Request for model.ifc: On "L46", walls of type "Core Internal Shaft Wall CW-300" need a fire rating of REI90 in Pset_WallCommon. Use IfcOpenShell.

First a look at what the model holds.

```python
import ifcopenshell
import ifcopenshell.util.element

model = ifcopenshell.open("model.ifc")
print(model.schema)
storey = next(s for s in model.by_type("IfcBuildingStorey") if s.Name == "L46")
walls = [e for e in ifcopenshell.util.element.get_decomposition(storey) if e.is_a("IfcWall")]
seen = {}
for e in walls:
    element_type = ifcopenshell.util.element.get_type(e)
    key = (element_type.Name if element_type != e and element_type else None, ifcopenshell.util.element.get_pset(e, "Pset_WallCommon", "FireRating"))
    seen[key] = seen.get(key, 0) + 1
for (name, value), count in sorted(seen.items(), key=str):
    print(count, "x", name, "|", value)
```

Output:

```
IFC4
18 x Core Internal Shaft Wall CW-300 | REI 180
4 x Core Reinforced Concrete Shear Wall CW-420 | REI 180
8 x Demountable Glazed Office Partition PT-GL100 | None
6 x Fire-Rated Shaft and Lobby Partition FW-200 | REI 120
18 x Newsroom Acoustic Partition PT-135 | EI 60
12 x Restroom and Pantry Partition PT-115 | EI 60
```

```python
import ifcopenshell
import ifcopenshell.api.pset
import ifcopenshell.util.element

model = ifcopenshell.open("model.ifc")

storey = next(s for s in model.by_type("IfcBuildingStorey") if s.Name == "L46")
walls = [e for e in ifcopenshell.util.element.get_decomposition(storey) if e.is_a("IfcWall")]

count = 0
for e in walls:
    element_type = ifcopenshell.util.element.get_type(e)
    if element_type in (None, e) or element_type.Name != "Core Internal Shaft Wall CW-300":
        continue
    found = ifcopenshell.util.element.get_pset(e, "Pset_WallCommon", should_inherit=False)
    if found:
        pset = model.by_id(found["id"])
        if len(ifcopenshell.util.element.get_elements_by_pset(pset)) > 1:
            pset = ifcopenshell.api.pset.unshare_pset(model, products=[e], pset=pset)[0]
    else:
        pset = ifcopenshell.api.pset.add_pset(model, product=e, name="Pset_WallCommon")
    ifcopenshell.api.pset.edit_pset(model, pset=pset, properties={"FireRating": "REI90"})
    count += 1

print(count, "walls updated")

model.write("model_edited.ifc")
```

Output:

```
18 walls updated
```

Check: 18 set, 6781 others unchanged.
